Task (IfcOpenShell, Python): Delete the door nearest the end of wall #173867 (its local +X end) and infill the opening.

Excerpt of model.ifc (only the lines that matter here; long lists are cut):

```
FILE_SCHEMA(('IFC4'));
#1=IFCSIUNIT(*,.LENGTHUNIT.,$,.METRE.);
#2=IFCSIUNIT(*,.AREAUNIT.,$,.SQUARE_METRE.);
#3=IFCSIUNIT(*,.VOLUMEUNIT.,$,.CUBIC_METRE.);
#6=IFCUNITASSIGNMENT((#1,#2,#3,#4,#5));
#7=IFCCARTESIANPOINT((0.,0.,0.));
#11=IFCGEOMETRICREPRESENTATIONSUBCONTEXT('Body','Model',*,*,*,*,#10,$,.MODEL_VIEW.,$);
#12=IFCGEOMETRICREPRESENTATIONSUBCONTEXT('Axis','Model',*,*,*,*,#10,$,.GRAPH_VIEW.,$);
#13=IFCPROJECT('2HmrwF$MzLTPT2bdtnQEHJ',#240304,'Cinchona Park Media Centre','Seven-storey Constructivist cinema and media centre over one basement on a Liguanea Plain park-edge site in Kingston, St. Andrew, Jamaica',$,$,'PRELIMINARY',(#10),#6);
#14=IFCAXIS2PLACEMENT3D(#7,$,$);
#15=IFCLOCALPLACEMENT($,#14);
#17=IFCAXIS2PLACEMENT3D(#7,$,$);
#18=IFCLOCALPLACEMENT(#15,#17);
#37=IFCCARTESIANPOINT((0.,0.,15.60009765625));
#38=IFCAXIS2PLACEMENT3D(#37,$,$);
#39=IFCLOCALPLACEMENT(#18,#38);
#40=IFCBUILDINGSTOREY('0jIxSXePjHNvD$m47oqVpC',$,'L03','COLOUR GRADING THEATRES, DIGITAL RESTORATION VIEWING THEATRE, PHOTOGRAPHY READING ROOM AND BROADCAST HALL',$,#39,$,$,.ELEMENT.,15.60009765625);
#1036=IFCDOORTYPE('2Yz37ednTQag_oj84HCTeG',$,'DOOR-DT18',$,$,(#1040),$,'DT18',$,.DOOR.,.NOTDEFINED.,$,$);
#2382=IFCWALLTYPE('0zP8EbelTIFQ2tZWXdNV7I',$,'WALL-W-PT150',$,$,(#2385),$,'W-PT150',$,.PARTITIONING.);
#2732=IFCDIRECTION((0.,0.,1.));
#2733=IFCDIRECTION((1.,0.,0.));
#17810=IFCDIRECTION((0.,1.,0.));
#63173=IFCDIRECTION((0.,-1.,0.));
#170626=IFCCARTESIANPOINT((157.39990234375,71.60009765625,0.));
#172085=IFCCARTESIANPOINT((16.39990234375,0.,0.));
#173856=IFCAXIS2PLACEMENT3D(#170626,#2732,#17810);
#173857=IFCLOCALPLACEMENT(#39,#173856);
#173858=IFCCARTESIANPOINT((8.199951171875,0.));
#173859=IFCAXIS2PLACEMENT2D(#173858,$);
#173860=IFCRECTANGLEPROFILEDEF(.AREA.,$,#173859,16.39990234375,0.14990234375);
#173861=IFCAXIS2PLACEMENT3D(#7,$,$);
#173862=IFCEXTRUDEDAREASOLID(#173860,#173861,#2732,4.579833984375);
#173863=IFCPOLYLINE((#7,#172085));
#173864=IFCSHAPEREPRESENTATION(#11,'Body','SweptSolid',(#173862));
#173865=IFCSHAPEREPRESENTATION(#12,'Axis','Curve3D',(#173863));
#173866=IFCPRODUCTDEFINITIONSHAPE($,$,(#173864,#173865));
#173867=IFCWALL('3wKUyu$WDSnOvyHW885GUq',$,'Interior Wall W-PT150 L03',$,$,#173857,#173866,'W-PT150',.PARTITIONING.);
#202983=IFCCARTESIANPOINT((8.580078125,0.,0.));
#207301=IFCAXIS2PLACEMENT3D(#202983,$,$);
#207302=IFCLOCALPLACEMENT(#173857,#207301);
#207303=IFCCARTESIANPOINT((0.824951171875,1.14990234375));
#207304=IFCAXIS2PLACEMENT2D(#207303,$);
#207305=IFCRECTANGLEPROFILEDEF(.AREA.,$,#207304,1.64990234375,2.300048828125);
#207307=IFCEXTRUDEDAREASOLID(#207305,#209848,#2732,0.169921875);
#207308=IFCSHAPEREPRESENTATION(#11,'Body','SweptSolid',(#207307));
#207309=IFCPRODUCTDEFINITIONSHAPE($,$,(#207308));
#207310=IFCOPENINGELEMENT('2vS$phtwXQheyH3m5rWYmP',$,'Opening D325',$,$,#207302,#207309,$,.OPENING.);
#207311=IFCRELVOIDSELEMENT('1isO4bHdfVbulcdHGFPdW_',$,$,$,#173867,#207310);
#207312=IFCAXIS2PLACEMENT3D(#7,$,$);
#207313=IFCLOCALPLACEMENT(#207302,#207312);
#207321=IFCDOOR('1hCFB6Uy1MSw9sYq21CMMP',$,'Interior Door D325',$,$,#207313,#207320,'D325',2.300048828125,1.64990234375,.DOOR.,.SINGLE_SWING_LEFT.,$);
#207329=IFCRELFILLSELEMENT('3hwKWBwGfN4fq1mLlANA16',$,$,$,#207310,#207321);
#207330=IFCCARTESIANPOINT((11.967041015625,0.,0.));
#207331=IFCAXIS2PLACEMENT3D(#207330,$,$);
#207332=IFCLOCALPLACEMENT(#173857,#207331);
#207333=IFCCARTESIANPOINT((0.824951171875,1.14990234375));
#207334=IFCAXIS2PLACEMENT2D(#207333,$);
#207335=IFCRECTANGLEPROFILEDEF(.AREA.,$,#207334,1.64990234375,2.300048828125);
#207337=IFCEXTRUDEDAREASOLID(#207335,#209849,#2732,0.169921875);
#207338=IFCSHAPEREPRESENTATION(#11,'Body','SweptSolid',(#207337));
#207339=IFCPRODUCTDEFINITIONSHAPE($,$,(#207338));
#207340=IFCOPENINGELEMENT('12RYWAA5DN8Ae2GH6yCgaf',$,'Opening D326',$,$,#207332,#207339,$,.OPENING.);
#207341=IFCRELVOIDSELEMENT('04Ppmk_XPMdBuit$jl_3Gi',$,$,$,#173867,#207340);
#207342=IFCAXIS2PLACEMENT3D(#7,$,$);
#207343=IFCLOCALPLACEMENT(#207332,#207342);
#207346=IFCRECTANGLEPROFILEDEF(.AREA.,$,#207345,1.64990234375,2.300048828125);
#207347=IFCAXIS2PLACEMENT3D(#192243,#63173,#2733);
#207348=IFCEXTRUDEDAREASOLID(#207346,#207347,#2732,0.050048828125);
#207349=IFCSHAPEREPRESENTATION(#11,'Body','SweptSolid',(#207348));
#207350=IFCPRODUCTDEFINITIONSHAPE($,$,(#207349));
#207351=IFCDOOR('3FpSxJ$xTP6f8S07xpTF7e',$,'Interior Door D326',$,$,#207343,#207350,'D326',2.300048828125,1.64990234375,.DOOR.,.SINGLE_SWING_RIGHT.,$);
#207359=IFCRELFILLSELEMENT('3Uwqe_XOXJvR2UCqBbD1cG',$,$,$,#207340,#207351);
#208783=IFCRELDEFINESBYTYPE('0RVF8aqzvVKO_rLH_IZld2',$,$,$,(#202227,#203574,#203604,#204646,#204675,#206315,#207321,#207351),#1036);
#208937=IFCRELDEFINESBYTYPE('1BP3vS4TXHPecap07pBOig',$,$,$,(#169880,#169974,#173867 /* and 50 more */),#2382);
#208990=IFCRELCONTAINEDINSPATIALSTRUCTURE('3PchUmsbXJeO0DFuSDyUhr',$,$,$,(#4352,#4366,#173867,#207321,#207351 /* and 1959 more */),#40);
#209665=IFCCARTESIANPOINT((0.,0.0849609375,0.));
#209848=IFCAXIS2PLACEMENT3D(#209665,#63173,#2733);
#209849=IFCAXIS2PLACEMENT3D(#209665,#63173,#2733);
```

```python
import ifcopenshell
import ifcopenshell.api.feature
import ifcopenshell.api.root
import ifcopenshell.geom
import ifcopenshell.util.shape

model = ifcopenshell.open("model.ifc")
settings = ifcopenshell.geom.settings()


def volume(element):
    """Net volume in cubic metres, openings subtracted."""
    shape = ifcopenshell.geom.create_shape(settings, element)
    return ifcopenshell.util.shape.get_volume(shape.geometry)


door = model.by_guid("3FpSxJ$xTP6f8S07xpTF7e")
opening = door.FillsVoids[0].RelatingOpeningElement
wall = opening.VoidsElements[0].RelatingBuildingElement
before = volume(wall)

ifcopenshell.api.root.remove_product(model, product=door)
ifcopenshell.api.feature.remove_feature(model, feature=opening)

after = volume(wall)

print(f"wall volume {before:.3f} -> {after:.3f} m3")

model.write("model_updated.ifc")
```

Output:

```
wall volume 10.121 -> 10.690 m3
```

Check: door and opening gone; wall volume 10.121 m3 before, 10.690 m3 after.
